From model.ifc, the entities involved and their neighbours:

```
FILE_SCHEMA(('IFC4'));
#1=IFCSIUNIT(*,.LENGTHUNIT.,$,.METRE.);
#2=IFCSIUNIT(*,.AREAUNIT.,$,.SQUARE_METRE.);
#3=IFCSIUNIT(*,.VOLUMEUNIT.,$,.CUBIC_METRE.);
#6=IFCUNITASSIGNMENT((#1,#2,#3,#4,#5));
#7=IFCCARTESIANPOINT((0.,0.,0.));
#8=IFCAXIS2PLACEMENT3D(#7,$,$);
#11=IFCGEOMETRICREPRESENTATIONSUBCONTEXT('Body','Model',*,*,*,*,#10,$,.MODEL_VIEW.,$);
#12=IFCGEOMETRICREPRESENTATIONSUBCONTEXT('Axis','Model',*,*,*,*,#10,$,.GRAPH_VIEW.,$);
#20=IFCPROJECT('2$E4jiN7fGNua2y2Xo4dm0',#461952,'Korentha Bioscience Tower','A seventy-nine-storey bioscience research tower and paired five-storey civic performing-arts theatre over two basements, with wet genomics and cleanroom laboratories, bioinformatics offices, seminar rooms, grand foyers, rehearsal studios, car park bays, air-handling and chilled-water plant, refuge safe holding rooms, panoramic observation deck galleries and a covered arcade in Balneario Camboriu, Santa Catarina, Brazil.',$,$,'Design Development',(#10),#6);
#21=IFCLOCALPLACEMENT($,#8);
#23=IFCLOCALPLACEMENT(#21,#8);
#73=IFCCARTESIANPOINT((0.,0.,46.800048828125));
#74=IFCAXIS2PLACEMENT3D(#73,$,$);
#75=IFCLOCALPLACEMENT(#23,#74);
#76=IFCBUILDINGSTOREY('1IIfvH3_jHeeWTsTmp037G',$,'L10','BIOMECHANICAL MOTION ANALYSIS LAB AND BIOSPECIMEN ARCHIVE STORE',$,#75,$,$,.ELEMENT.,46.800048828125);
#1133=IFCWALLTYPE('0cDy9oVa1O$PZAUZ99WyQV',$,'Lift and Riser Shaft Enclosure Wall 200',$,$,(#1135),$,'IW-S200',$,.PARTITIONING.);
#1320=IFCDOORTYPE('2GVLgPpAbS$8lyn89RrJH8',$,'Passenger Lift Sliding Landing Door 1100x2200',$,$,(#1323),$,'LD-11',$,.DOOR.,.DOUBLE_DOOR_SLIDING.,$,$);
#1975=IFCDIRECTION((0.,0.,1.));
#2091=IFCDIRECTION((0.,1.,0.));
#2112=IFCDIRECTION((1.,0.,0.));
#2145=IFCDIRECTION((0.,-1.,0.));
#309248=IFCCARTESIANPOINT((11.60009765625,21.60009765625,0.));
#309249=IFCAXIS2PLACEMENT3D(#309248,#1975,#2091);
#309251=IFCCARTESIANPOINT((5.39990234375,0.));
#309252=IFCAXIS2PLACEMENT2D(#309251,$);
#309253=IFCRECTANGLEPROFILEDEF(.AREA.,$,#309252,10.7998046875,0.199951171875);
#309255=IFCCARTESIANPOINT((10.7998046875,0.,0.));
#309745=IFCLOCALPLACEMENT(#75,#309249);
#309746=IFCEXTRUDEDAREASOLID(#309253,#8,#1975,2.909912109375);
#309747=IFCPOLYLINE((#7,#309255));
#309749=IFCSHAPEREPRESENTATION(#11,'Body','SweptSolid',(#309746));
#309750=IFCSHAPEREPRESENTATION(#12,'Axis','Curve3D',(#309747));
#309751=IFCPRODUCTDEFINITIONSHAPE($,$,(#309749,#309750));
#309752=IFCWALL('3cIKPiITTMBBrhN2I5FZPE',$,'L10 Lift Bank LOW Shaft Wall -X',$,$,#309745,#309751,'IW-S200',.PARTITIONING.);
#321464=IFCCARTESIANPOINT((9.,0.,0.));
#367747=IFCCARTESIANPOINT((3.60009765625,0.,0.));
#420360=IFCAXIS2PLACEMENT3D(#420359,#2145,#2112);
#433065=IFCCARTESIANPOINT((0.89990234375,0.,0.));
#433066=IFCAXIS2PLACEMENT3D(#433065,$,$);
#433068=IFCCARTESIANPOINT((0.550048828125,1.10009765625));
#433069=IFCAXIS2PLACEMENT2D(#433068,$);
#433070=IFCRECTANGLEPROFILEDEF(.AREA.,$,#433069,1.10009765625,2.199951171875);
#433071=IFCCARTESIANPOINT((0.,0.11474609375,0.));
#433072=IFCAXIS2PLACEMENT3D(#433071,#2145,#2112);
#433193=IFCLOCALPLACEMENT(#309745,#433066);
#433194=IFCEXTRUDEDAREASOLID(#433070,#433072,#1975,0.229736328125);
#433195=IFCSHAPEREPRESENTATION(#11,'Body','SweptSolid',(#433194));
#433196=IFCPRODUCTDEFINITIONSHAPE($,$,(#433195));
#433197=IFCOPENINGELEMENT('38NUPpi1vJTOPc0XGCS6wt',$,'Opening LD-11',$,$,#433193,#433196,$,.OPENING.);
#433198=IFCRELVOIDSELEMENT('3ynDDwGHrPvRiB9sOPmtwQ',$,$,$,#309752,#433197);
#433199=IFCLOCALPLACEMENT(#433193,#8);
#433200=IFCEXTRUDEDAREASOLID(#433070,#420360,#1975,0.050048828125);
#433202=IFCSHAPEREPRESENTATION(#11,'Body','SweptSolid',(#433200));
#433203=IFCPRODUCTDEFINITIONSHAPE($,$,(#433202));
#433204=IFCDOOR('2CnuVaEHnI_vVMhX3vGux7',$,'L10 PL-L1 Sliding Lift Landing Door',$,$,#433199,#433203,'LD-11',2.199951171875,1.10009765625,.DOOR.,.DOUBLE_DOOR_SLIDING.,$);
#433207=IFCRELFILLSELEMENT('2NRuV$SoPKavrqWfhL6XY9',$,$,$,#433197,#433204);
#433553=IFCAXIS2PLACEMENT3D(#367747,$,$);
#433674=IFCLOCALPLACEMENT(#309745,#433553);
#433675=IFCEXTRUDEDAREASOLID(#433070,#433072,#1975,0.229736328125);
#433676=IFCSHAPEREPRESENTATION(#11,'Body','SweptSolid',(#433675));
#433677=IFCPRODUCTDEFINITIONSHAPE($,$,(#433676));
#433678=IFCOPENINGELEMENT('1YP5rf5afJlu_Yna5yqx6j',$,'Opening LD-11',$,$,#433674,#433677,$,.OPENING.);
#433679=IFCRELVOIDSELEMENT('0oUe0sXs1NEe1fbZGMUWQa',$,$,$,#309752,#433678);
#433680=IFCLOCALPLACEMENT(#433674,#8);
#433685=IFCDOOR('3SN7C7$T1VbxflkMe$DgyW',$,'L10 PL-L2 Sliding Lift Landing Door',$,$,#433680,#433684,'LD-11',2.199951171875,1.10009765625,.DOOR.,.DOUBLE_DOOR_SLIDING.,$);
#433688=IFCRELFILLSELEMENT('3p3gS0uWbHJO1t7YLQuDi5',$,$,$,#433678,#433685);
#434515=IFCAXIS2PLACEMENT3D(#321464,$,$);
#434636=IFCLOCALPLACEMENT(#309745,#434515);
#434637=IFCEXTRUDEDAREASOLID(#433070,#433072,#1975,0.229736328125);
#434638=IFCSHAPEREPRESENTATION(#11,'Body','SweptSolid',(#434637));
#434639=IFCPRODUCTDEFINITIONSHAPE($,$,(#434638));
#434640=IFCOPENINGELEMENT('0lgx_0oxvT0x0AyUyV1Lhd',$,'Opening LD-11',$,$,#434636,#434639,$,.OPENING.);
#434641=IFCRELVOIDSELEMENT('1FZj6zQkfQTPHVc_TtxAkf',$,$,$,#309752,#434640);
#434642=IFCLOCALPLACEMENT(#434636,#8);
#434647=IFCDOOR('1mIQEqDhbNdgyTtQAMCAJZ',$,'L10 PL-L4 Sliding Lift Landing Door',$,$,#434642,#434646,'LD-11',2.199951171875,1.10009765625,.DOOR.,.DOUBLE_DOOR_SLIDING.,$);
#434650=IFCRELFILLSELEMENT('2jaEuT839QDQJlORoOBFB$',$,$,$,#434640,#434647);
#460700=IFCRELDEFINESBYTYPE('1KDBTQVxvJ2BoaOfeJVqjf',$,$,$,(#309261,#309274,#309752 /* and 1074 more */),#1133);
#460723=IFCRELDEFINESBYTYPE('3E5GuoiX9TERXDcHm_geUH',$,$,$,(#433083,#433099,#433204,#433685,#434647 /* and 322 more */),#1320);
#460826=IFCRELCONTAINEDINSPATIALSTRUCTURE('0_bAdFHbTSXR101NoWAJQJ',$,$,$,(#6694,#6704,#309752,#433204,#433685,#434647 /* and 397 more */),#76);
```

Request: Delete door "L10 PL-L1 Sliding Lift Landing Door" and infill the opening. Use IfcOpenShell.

```python
import ifcopenshell
import ifcopenshell.api.feature
import ifcopenshell.api.root
import ifcopenshell.geom
import ifcopenshell.util.shape

model = ifcopenshell.open("model.ifc")
settings = ifcopenshell.geom.settings()


def volume(element):
    """Net volume in cubic metres, openings subtracted."""
    shape = ifcopenshell.geom.create_shape(settings, element)
    return ifcopenshell.util.shape.get_volume(shape.geometry)


door = model.by_guid("2CnuVaEHnI_vVMhX3vGux7")
opening = door.FillsVoids[0].RelatingOpeningElement
wall = opening.VoidsElements[0].RelatingBuildingElement
before = volume(wall)

ifcopenshell.api.root.remove_product(model, product=door)
ifcopenshell.api.feature.remove_feature(model, feature=opening)

after = volume(wall)

print(f"wall volume {before:.3f} -> {after:.3f} m3")

model.write("model_edited.ifc")
```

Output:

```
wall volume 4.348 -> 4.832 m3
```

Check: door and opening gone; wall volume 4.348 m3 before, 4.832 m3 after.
